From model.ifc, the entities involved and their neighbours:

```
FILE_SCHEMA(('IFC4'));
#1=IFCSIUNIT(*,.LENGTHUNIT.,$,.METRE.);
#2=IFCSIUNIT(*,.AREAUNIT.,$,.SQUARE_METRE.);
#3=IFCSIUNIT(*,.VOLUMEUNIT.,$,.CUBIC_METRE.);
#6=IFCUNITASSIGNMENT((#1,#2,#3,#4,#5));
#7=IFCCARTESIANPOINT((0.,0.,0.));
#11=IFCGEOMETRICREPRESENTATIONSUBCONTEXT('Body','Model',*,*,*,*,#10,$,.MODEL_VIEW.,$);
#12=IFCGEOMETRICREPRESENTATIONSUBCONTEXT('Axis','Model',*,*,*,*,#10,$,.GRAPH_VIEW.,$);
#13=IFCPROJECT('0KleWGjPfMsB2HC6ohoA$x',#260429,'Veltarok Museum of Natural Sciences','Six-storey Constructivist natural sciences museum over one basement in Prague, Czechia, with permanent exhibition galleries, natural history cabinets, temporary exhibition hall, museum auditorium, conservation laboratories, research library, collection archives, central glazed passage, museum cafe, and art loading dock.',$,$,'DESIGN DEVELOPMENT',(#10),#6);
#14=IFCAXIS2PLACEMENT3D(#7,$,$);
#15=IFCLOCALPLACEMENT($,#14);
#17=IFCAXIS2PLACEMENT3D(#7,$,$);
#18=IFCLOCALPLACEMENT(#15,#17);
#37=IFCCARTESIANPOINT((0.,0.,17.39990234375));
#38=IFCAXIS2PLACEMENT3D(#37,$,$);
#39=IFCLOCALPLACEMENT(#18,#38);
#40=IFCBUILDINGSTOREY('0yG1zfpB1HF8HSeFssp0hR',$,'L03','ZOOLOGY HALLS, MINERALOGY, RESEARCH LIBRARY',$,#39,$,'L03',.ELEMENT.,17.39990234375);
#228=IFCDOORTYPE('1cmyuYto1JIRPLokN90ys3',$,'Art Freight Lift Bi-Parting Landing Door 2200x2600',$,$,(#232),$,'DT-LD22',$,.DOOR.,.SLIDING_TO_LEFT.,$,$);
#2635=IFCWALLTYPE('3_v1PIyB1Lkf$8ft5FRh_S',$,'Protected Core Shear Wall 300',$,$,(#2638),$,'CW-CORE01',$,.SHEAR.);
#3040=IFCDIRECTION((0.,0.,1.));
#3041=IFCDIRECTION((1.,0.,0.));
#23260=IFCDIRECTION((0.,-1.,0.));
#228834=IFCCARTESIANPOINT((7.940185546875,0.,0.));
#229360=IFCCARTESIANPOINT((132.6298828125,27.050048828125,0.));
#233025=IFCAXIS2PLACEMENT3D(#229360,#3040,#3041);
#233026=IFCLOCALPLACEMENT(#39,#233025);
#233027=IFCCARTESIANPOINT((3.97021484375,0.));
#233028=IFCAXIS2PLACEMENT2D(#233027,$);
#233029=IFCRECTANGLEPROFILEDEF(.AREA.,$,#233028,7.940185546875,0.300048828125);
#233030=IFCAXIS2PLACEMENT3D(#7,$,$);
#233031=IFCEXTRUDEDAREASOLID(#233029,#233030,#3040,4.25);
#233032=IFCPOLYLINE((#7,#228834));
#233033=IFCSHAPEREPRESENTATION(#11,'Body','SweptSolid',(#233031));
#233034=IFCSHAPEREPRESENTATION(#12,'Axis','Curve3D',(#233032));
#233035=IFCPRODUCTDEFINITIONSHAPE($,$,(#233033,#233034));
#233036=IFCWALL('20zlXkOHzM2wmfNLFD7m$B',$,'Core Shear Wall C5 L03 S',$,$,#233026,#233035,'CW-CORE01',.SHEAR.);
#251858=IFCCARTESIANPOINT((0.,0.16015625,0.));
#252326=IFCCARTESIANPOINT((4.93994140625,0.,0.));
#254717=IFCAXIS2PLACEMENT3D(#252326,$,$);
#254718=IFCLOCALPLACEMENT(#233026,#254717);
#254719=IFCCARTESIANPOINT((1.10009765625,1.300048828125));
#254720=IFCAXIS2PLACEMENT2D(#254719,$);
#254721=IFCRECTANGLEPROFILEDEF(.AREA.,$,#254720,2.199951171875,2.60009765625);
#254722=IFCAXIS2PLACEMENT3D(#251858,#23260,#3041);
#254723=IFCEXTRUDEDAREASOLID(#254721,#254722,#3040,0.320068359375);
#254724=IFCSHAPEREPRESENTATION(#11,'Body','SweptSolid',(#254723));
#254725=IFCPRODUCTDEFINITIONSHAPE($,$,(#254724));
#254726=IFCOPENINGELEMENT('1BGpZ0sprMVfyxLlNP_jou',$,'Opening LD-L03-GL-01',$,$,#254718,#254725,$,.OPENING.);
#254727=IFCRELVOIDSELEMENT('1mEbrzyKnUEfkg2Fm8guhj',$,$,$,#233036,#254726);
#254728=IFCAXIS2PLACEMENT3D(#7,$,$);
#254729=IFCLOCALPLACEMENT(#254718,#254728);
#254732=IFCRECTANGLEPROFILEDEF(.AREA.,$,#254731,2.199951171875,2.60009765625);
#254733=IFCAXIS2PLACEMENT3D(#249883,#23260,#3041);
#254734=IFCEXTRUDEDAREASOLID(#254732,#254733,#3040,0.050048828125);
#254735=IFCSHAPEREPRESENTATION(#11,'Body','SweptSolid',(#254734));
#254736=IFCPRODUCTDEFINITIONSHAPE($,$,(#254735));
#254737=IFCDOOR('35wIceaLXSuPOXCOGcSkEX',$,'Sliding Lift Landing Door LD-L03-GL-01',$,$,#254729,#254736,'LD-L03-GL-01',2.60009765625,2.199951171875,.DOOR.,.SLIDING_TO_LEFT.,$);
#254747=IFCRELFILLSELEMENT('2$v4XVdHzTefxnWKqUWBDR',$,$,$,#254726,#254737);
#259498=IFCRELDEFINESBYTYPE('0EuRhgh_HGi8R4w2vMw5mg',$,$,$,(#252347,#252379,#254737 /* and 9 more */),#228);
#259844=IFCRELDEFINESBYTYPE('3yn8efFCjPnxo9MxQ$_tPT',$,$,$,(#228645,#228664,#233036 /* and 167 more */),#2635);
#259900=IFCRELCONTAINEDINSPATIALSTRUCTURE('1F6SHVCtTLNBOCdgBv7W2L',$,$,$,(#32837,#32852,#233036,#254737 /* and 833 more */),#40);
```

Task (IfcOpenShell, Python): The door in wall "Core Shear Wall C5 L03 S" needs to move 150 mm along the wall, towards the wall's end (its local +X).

```python
import ifcopenshell
import ifcopenshell.api.geometry
import ifcopenshell.util.placement

model = ifcopenshell.open("model.ifc")

door = model.by_guid("35wIceaLXSuPOXCOGcSkEX")
opening = door.FillsVoids[0].RelatingOpeningElement
wall = opening.VoidsElements[0].RelatingBuildingElement

wall_matrix = ifcopenshell.util.placement.get_local_placement(wall.ObjectPlacement)
shift = wall_matrix[:3, 0] * 0.15
before = ifcopenshell.util.placement.get_local_placement(door.ObjectPlacement)[:3, 3].copy()

# The door is placed relative to its opening, so it follows when the opening moves.
matrix = ifcopenshell.util.placement.get_local_placement(opening.ObjectPlacement)
matrix[:3, 3] += shift
ifcopenshell.api.geometry.edit_object_placement(
    model, product=opening, matrix=matrix, is_si=False, should_transform_children=True
)

after = ifcopenshell.util.placement.get_local_placement(door.ObjectPlacement)[:3, 3]
print("door moved by", (after - before).round(3) + 0.0)

model.write("model_rev.ifc")
```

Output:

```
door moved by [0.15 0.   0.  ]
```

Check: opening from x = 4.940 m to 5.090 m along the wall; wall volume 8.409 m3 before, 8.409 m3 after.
